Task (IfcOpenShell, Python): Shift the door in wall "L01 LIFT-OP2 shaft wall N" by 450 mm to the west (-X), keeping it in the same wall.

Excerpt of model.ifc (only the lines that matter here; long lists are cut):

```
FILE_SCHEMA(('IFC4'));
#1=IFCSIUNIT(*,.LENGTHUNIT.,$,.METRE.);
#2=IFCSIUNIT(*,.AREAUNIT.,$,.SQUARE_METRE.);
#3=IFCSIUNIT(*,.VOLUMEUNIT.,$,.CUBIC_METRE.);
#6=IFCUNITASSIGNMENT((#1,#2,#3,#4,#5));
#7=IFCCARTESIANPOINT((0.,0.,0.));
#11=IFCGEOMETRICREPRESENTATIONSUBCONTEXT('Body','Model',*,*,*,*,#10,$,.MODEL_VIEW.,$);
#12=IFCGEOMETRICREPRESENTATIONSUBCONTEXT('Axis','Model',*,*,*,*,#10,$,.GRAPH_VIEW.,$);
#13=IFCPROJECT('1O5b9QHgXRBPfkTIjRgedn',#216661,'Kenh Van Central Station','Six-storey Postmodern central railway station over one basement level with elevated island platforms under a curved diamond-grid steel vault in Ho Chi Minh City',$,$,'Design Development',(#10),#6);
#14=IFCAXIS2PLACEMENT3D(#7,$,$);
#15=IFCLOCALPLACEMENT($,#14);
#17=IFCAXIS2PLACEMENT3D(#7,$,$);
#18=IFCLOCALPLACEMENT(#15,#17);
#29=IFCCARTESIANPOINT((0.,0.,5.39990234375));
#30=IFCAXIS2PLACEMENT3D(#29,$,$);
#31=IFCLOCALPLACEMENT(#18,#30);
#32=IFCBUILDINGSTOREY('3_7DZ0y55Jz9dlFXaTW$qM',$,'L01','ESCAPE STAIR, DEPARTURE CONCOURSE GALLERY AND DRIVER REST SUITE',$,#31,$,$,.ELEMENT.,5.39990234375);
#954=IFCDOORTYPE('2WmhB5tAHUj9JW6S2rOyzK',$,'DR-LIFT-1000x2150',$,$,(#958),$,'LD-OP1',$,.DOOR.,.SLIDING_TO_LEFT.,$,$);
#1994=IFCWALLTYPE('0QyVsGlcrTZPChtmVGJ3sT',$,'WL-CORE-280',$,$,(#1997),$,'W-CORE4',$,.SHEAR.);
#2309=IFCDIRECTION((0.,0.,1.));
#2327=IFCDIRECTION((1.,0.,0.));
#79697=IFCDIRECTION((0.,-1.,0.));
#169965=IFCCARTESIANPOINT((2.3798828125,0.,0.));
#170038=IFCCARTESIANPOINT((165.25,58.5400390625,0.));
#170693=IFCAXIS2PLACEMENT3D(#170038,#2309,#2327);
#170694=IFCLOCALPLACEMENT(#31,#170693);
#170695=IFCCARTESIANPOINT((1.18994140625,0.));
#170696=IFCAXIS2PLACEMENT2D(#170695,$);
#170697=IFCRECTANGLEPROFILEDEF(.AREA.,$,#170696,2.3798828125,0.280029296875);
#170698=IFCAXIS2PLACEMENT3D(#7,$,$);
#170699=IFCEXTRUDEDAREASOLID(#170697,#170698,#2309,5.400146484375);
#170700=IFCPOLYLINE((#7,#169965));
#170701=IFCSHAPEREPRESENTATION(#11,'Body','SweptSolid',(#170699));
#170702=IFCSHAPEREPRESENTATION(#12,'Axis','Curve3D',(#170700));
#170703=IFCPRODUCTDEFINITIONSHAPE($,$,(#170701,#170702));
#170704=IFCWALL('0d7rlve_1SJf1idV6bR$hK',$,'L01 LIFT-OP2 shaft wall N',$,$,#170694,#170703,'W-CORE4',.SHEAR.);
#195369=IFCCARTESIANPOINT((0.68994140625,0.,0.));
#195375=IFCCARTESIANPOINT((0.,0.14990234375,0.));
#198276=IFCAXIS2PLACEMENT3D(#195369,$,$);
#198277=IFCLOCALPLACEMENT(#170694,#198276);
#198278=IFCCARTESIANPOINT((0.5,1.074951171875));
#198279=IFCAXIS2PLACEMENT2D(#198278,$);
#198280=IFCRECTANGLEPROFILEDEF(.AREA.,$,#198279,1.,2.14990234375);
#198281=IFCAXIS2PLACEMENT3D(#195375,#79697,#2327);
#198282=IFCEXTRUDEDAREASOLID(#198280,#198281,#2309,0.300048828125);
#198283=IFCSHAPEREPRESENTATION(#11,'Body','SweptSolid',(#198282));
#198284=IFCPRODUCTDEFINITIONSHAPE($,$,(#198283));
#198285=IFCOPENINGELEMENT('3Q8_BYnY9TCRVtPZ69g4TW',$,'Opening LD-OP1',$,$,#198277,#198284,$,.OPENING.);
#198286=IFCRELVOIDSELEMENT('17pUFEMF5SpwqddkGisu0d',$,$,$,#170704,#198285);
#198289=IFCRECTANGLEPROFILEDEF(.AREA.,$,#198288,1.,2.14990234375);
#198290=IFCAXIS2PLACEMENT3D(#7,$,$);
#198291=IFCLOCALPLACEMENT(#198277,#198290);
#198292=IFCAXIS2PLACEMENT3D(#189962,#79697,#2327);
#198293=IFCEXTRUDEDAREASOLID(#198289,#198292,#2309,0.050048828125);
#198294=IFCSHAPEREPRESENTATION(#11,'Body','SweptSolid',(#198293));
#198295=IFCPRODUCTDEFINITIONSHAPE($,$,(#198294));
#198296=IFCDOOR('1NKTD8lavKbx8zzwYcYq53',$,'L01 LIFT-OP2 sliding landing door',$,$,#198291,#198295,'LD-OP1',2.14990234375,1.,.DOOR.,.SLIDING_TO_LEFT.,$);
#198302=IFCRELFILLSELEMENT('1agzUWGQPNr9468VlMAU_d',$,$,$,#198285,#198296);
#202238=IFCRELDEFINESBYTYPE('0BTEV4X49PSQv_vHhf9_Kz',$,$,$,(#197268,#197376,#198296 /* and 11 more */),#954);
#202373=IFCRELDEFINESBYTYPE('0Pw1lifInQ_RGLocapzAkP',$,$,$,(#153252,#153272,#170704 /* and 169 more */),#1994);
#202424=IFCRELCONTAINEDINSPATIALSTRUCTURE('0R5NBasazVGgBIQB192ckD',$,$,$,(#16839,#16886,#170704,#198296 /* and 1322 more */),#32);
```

```python
import ifcopenshell
import ifcopenshell.api.geometry
import ifcopenshell.util.placement
import ifcopenshell.util.unit

model = ifcopenshell.open("model.ifc")
unit_scale = ifcopenshell.util.unit.calculate_unit_scale(model)

door = model.by_guid("1NKTD8lavKbx8zzwYcYq53")
opening = door.FillsVoids[0].RelatingOpeningElement
wall = opening.VoidsElements[0].RelatingBuildingElement

wall_matrix = ifcopenshell.util.placement.get_local_placement(wall.ObjectPlacement)
shift = wall_matrix[:3, 0] * -0.45 / unit_scale
before = ifcopenshell.util.placement.get_local_placement(door.ObjectPlacement)[:3, 3].copy()

# The door is placed relative to its opening, so it follows when the opening moves.
matrix = ifcopenshell.util.placement.get_local_placement(opening.ObjectPlacement)
matrix[:3, 3] += shift
ifcopenshell.api.geometry.edit_object_placement(
    model, product=opening, matrix=matrix, is_si=False, should_transform_children=True
)

after = ifcopenshell.util.placement.get_local_placement(door.ObjectPlacement)[:3, 3]
print("door moved by", (after - before).round(3) + 0.0)

model.write("model_edited.ifc")
```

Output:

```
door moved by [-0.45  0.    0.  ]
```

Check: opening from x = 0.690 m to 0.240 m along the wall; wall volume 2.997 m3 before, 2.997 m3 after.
